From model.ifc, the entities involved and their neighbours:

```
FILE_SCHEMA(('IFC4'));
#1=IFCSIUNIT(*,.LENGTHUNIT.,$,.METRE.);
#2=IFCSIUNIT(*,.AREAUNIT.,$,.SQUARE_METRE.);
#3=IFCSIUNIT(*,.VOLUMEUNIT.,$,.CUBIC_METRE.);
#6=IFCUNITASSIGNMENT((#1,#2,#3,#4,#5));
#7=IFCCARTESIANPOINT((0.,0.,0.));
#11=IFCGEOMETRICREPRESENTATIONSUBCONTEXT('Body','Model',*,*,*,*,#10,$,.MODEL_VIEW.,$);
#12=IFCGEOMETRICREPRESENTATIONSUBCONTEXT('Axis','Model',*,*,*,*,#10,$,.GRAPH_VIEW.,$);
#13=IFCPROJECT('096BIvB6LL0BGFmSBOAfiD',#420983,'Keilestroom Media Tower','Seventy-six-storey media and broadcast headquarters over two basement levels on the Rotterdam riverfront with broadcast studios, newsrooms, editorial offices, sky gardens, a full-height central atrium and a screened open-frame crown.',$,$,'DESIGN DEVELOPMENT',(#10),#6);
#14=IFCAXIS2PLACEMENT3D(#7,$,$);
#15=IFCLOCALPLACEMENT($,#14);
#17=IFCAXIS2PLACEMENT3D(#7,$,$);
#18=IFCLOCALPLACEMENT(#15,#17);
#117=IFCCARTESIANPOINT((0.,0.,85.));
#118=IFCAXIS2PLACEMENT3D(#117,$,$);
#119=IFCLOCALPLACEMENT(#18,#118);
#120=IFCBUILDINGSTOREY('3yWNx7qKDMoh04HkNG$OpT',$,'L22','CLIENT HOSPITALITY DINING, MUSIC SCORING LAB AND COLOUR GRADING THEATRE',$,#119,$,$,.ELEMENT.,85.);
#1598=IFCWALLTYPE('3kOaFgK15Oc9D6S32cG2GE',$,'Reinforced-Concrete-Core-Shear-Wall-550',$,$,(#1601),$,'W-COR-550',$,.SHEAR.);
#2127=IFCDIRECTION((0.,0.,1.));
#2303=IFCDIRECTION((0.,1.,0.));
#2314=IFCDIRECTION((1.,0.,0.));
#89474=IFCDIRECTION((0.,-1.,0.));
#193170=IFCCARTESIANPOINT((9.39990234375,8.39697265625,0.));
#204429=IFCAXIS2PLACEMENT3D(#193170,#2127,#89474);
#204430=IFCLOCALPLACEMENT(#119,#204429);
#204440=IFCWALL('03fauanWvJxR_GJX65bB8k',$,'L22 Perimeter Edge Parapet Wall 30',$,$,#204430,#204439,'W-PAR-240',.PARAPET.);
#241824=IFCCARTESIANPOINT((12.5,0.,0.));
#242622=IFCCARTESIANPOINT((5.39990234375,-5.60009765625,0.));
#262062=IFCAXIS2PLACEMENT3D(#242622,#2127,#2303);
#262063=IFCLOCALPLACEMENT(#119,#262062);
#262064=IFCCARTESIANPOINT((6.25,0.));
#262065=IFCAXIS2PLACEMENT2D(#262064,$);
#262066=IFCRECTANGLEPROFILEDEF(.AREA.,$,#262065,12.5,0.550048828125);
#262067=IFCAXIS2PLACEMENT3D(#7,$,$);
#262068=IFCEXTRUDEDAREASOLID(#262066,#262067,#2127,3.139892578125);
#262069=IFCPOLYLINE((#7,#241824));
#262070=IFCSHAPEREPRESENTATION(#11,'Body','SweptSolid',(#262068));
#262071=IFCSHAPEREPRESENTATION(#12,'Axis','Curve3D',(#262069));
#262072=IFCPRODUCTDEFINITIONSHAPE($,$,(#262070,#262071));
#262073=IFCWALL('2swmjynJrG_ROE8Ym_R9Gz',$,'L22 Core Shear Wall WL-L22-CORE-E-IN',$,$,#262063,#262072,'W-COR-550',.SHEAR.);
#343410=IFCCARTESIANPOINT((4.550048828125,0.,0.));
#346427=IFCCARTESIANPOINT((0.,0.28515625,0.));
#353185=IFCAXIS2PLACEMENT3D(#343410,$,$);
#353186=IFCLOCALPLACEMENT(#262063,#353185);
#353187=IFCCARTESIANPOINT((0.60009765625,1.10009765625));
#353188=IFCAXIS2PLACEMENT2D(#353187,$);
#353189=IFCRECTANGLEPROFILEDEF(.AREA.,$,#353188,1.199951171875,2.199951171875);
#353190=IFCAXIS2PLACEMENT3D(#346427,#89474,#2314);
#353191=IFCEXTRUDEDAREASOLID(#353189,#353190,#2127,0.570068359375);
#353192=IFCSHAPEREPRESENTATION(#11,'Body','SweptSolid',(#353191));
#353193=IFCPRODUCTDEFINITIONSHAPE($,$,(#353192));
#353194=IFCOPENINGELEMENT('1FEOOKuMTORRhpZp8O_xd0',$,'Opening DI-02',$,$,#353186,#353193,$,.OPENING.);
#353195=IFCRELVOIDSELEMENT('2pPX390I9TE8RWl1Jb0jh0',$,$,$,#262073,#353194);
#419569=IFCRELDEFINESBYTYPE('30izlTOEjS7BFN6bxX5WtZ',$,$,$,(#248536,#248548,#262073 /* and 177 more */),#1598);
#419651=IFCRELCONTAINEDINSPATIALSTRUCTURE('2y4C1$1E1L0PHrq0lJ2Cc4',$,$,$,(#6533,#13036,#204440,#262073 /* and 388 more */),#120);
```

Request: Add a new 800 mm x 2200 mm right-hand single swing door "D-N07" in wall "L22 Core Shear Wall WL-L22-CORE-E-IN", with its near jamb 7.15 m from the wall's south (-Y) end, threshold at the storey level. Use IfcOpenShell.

```python
import numpy as np
import ifcopenshell
import ifcopenshell.api.feature
import ifcopenshell.api.geometry
import ifcopenshell.api.root
import ifcopenshell.api.spatial
import ifcopenshell.geom
import ifcopenshell.util.element
import ifcopenshell.util.placement
import ifcopenshell.util.representation
import ifcopenshell.util.shape
import ifcopenshell.util.unit

model = ifcopenshell.open("model.ifc")
unit_scale = ifcopenshell.util.unit.calculate_unit_scale(model)
settings = ifcopenshell.geom.settings()


def volume(element):
    """Net volume in cubic metres, openings subtracted."""
    shape = ifcopenshell.geom.create_shape(settings, element)
    return ifcopenshell.util.shape.get_volume(shape.geometry)


wall = model.by_guid("2swmjynJrG_ROE8Ym_R9Gz")
storey = ifcopenshell.util.element.get_container(wall, ifc_class="IfcBuildingStorey")
context = ifcopenshell.util.representation.get_context(model, "Model", "Body", "MODEL_VIEW")
before = volume(wall)

width, height, from_end, sill = 0.8, 2.2, 7.15, 0.0  # metres

# The wall runs along its own X axis, and the end named is its -X end.
wall_shape = ifcopenshell.geom.create_shape(settings, wall)
x, y, z = ifcopenshell.util.shape.get_vertices(wall_shape.geometry).T
start = x.min() + from_end
face, thickness = float(y.min()), float(y.max() - y.min())
wall_matrix = ifcopenshell.util.placement.get_local_placement(wall.ObjectPlacement)
level = ifcopenshell.util.placement.get_local_placement(storey.ObjectPlacement)[2, 3]


def in_wall(x, y):
    """Placement at x, y metres in the wall's axes, at sill height."""
    matrix = wall_matrix.copy()
    matrix[:, 3] = wall_matrix @ np.array([x / unit_scale, y / unit_scale, 0.0, 1.0])
    matrix[2, 3] = level + sill / unit_scale
    return matrix


# Opening: a box that overshoots both wall faces by 50 mm.
opening = ifcopenshell.api.root.create_entity(model, ifc_class="IfcOpeningElement", predefined_type="OPENING")
box = ifcopenshell.api.geometry.add_wall_representation(
    model, context=context, length=width, height=height, thickness=thickness + 0.1
)
ifcopenshell.api.geometry.assign_representation(model, product=opening, representation=box)
ifcopenshell.api.geometry.edit_object_placement(model, product=opening, matrix=in_wall(start, face - 0.05), is_si=False)
ifcopenshell.api.feature.add_feature(model, feature=opening, element=wall)

door = ifcopenshell.api.root.create_entity(model, ifc_class="IfcDoor", name="D-N07", predefined_type="DOOR")
door.OverallWidth, door.OverallHeight = width / unit_scale, height / unit_scale
door.OperationType = "SINGLE_SWING_RIGHT"
body = ifcopenshell.api.geometry.add_door_representation(
    model,
    context=context,
    overall_width=door.OverallWidth,
    overall_height=door.OverallHeight,
    operation_type="SINGLE_SWING_RIGHT",
    lining_properties={"LiningDepth": thickness / unit_scale, "ThresholdDepth": thickness / unit_scale},
)
ifcopenshell.api.geometry.assign_representation(model, product=door, representation=body)
ifcopenshell.api.spatial.assign_container(model, products=[door], relating_structure=storey)
ifcopenshell.api.feature.add_filling(model, opening=opening, element=door)

# The lining spans the wall, so the door starts at the wall face.
ifcopenshell.api.geometry.edit_object_placement(model, product=door, matrix=in_wall(start, face), is_si=False)

after = volume(wall)

print(f"wall volume {before:.3f} -> {after:.3f} m3")

model.write("model_updated.ifc")
```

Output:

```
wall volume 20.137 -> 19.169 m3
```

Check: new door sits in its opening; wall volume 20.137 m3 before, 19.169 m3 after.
